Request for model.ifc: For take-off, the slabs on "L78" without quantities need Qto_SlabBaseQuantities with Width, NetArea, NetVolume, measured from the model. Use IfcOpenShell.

First a look at what the model holds.

```python
import ifcopenshell
import ifcopenshell.util.element
import ifcopenshell.util.unit

model = ifcopenshell.open("model.ifc")
print(model.schema)
for unit_type in ("LENGTHUNIT", "AREAUNIT", "VOLUMEUNIT"):
    print(unit_type, ifcopenshell.util.unit.calculate_unit_scale(model, unit_type))
storey = next(s for s in model.by_type("IfcBuildingStorey") if s.Name == "L78")
slabs = [e for e in ifcopenshell.util.element.get_decomposition(storey) if e.is_a("IfcSlab")]
for e in sorted(slabs, key=lambda e: e.id()):
    print(e.id(), e.is_a(), e.Name, list(ifcopenshell.util.element.get_psets(e, qtos_only=True)), sep=" | ")
```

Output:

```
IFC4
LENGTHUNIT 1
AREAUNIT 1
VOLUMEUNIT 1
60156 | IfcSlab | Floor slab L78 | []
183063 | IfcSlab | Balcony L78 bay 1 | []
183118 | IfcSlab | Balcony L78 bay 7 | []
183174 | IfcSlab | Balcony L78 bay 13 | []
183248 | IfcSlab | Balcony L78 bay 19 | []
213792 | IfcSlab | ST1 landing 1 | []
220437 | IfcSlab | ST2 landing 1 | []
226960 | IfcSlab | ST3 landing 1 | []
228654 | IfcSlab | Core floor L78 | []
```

```python
import ifcopenshell
import ifcopenshell.api.pset
import ifcopenshell.geom
import ifcopenshell.util.element
import ifcopenshell.util.shape
import ifcopenshell.util.unit

model = ifcopenshell.open("model.ifc")
unit_scale = ifcopenshell.util.unit.calculate_unit_scale(model)
area_scale = ifcopenshell.util.unit.calculate_unit_scale(model, "AREAUNIT")
volume_scale = ifcopenshell.util.unit.calculate_unit_scale(model, "VOLUMEUNIT")
settings = ifcopenshell.geom.settings()

storey = next(s for s in model.by_type("IfcBuildingStorey") if s.Name == "L78")
slabs = [e for e in ifcopenshell.util.element.get_decomposition(storey) if e.is_a("IfcSlab")]

for e in sorted(slabs, key=lambda e: e.id()):
    if ifcopenshell.util.element.get_psets(e, qtos_only=True, should_inherit=False):
        continue
    # Geometry comes back in metres, in the element's own axes.
    shape = ifcopenshell.geom.create_shape(settings, e)
    values = {
        "Width": ifcopenshell.util.shape.get_z(shape.geometry) / unit_scale,
        "NetArea": ifcopenshell.util.shape.get_footprint_area(shape.geometry) / area_scale,
        "NetVolume": ifcopenshell.util.shape.get_volume(shape.geometry) / volume_scale,
    }
    qto = ifcopenshell.api.pset.add_qto(model, product=e, name="Qto_SlabBaseQuantities")
    ifcopenshell.api.pset.edit_qto(model, qto=qto, properties=values)
    print(e.id(), {k: round(v, 3) for k, v in values.items()})

model.write("model_edited.ifc")
```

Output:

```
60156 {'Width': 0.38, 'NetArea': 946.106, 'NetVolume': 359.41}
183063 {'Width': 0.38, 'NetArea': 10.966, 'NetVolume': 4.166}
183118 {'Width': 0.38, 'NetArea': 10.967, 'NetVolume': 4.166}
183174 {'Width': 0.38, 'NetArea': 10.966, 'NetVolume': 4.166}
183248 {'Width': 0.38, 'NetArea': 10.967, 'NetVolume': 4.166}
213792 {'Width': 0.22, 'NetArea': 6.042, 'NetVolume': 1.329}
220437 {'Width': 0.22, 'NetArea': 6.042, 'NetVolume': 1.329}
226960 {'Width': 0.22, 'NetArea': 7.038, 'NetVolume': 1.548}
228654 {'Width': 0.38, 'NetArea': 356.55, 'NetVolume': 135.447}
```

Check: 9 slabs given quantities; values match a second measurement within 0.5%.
